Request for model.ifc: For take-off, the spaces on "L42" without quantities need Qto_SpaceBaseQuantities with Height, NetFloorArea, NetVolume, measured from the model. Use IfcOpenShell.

First a look at what the model holds.

```python
import ifcopenshell
import ifcopenshell.util.element
import ifcopenshell.util.unit

model = ifcopenshell.open("model.ifc")
print(model.schema)
for unit_type in ("LENGTHUNIT", "AREAUNIT", "VOLUMEUNIT"):
    print(unit_type, ifcopenshell.util.unit.calculate_unit_scale(model, unit_type))
storey = next(s for s in model.by_type("IfcBuildingStorey") if s.Name == "L42")
spaces = [e for e in ifcopenshell.util.element.get_decomposition(storey) if e.is_a("IfcSpace")]
for e in sorted(spaces, key=lambda e: e.id()):
    print(e.id(), e.is_a(), e.Name, list(ifcopenshell.util.element.get_psets(e, qtos_only=True)), sep=" | ")
```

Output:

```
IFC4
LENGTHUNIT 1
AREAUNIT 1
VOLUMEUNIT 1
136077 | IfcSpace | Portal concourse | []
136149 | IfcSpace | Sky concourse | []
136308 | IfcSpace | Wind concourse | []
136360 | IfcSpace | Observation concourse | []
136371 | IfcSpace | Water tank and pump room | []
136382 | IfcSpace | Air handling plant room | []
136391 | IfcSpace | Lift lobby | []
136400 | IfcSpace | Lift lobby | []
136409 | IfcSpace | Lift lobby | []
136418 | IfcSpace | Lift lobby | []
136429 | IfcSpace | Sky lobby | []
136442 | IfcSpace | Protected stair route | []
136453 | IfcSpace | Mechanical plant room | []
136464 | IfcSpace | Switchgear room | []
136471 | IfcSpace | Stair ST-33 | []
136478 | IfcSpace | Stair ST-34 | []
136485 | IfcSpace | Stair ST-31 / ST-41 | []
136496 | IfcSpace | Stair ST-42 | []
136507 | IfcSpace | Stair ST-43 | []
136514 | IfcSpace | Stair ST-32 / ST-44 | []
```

```python
import ifcopenshell
import ifcopenshell.api.pset
import ifcopenshell.geom
import ifcopenshell.util.element
import ifcopenshell.util.shape
import ifcopenshell.util.unit

model = ifcopenshell.open("model.ifc")
unit_scale = ifcopenshell.util.unit.calculate_unit_scale(model)
area_scale = ifcopenshell.util.unit.calculate_unit_scale(model, "AREAUNIT")
volume_scale = ifcopenshell.util.unit.calculate_unit_scale(model, "VOLUMEUNIT")
settings = ifcopenshell.geom.settings()

storey = next(s for s in model.by_type("IfcBuildingStorey") if s.Name == "L42")
spaces = [e for e in ifcopenshell.util.element.get_decomposition(storey) if e.is_a("IfcSpace")]

for e in sorted(spaces, key=lambda e: e.id()):
    if ifcopenshell.util.element.get_psets(e, qtos_only=True, should_inherit=False):
        continue
    # Geometry comes back in metres, in the element's own axes.
    shape = ifcopenshell.geom.create_shape(settings, e)
    values = {
        "Height": ifcopenshell.util.shape.get_z(shape.geometry) / unit_scale,
        "NetFloorArea": ifcopenshell.util.shape.get_footprint_area(shape.geometry) / area_scale,
        "NetVolume": ifcopenshell.util.shape.get_volume(shape.geometry) / volume_scale,
    }
    qto = ifcopenshell.api.pset.add_qto(model, product=e, name="Qto_SpaceBaseQuantities")
    ifcopenshell.api.pset.edit_qto(model, qto=qto, properties=values)
    print(e.id(), {k: round(v, 3) for k, v in values.items()})

model.write("model_v2.ifc")
```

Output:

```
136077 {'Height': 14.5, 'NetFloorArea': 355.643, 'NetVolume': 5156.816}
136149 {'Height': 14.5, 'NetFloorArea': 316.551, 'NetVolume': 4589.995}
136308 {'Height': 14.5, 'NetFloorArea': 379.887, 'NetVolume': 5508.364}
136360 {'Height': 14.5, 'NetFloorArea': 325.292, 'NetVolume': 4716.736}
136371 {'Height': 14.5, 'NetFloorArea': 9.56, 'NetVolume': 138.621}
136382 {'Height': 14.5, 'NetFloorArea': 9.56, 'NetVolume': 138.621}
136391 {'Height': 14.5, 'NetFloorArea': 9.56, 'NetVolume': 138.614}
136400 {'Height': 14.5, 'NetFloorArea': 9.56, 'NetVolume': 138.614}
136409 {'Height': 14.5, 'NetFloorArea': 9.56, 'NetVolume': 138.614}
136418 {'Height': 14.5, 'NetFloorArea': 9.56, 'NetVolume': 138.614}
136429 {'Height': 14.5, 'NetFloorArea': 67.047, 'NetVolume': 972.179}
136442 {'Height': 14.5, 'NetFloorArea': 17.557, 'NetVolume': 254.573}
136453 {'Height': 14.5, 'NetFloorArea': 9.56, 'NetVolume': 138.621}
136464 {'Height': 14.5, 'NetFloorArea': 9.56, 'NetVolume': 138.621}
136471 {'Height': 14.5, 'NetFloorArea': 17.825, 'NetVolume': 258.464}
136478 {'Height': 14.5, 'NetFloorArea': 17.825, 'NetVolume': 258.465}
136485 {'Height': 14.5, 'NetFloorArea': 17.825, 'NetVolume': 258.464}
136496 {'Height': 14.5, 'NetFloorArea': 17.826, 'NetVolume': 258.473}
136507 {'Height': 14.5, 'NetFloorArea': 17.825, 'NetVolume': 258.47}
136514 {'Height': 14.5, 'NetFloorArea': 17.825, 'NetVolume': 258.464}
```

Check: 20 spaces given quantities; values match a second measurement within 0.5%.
